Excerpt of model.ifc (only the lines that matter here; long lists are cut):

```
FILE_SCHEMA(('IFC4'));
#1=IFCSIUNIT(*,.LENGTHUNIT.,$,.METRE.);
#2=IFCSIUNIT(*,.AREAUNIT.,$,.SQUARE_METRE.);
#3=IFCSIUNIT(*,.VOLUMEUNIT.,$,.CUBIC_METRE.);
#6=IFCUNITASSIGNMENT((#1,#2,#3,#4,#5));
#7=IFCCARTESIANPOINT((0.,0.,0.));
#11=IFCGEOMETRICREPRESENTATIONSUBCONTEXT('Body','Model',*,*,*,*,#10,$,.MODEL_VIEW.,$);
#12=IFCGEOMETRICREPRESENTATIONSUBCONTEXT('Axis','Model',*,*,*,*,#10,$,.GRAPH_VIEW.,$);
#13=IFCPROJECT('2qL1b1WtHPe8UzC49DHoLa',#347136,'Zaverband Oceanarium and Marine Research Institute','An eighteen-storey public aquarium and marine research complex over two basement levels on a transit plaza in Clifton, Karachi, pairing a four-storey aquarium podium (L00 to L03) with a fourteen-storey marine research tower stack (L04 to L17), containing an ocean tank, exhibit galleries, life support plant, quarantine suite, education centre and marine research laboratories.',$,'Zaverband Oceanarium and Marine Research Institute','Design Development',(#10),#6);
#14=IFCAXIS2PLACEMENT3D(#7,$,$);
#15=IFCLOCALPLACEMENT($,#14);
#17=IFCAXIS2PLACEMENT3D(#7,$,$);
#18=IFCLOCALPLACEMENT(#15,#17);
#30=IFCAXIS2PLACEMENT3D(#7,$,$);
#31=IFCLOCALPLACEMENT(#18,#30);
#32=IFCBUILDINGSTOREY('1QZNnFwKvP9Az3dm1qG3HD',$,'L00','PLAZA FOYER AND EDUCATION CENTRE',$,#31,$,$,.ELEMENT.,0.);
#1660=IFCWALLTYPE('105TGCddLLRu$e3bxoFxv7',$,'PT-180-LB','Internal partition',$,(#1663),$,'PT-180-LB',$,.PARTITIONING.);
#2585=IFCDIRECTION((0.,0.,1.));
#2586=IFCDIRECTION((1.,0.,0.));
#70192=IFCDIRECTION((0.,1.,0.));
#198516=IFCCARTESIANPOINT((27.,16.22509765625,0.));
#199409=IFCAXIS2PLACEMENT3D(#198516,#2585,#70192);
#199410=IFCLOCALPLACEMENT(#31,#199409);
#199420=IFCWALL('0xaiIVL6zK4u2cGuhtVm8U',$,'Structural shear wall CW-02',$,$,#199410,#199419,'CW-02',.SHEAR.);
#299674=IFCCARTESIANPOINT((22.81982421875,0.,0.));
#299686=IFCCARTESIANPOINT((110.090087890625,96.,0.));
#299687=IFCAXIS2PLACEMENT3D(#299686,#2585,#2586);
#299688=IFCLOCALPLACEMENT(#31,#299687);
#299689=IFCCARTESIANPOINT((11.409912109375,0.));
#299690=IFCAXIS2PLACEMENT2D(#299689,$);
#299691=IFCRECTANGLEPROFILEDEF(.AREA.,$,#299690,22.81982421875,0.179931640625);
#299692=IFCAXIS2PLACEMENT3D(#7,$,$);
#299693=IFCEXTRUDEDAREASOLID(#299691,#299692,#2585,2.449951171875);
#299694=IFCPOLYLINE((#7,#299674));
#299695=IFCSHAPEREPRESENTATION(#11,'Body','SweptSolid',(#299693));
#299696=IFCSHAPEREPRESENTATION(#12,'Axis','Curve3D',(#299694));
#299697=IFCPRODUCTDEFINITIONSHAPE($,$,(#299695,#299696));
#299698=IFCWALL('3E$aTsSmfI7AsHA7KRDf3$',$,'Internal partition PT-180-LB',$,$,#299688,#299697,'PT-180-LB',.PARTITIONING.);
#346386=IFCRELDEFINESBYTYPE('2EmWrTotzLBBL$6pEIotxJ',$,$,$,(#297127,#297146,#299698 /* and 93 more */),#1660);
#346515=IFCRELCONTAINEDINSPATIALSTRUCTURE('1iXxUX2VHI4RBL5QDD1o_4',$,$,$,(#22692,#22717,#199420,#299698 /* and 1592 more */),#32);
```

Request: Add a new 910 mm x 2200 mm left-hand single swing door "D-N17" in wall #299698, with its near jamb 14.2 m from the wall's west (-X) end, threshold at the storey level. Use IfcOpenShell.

```python
import numpy as np
import ifcopenshell
import ifcopenshell.api.feature
import ifcopenshell.api.geometry
import ifcopenshell.api.root
import ifcopenshell.api.spatial
import ifcopenshell.geom
import ifcopenshell.util.element
import ifcopenshell.util.placement
import ifcopenshell.util.representation
import ifcopenshell.util.shape
import ifcopenshell.util.unit

model = ifcopenshell.open("model.ifc")
unit_scale = ifcopenshell.util.unit.calculate_unit_scale(model)
settings = ifcopenshell.geom.settings()


def volume(element):
    """Net volume in cubic metres, openings subtracted."""
    shape = ifcopenshell.geom.create_shape(settings, element)
    return ifcopenshell.util.shape.get_volume(shape.geometry)


wall = model.by_guid("3E$aTsSmfI7AsHA7KRDf3$")
storey = ifcopenshell.util.element.get_container(wall, ifc_class="IfcBuildingStorey")
context = ifcopenshell.util.representation.get_context(model, "Model", "Body", "MODEL_VIEW")
before = volume(wall)

width, height, from_end, sill = 0.91, 2.2, 14.2, 0.0  # metres

# The wall runs along its own X axis, and the end named is its -X end.
wall_shape = ifcopenshell.geom.create_shape(settings, wall)
x, y, z = ifcopenshell.util.shape.get_vertices(wall_shape.geometry).T
start = x.min() + from_end
face, thickness = float(y.min()), float(y.max() - y.min())
wall_matrix = ifcopenshell.util.placement.get_local_placement(wall.ObjectPlacement)
level = ifcopenshell.util.placement.get_local_placement(storey.ObjectPlacement)[2, 3]


def in_wall(x, y):
    """Placement at x, y metres in the wall's axes, at sill height."""
    matrix = wall_matrix.copy()
    matrix[:, 3] = wall_matrix @ np.array([x / unit_scale, y / unit_scale, 0.0, 1.0])
    matrix[2, 3] = level + sill / unit_scale
    return matrix


# Opening: a box that overshoots both wall faces by 50 mm.
opening = ifcopenshell.api.root.create_entity(model, ifc_class="IfcOpeningElement", predefined_type="OPENING")
box = ifcopenshell.api.geometry.add_wall_representation(
    model, context=context, length=width, height=height, thickness=thickness + 0.1
)
ifcopenshell.api.geometry.assign_representation(model, product=opening, representation=box)
ifcopenshell.api.geometry.edit_object_placement(model, product=opening, matrix=in_wall(start, face - 0.05), is_si=False)
ifcopenshell.api.feature.add_feature(model, feature=opening, element=wall)

door = ifcopenshell.api.root.create_entity(model, ifc_class="IfcDoor", name="D-N17", predefined_type="DOOR")
door.OverallWidth, door.OverallHeight = width / unit_scale, height / unit_scale
door.OperationType = "SINGLE_SWING_LEFT"
body = ifcopenshell.api.geometry.add_door_representation(
    model,
    context=context,
    overall_width=door.OverallWidth,
    overall_height=door.OverallHeight,
    operation_type="SINGLE_SWING_LEFT",
    lining_properties={"LiningDepth": thickness / unit_scale, "ThresholdDepth": thickness / unit_scale},
)
ifcopenshell.api.geometry.assign_representation(model, product=door, representation=body)
ifcopenshell.api.spatial.assign_container(model, products=[door], relating_structure=storey)
ifcopenshell.api.feature.add_filling(model, opening=opening, element=door)

# The lining spans the wall, so the door starts at the wall face.
ifcopenshell.api.geometry.edit_object_placement(model, product=door, matrix=in_wall(start, face), is_si=False)

after = volume(wall)

print(f"wall volume {before:.3f} -> {after:.3f} m3")

model.write("model_edited.ifc")
```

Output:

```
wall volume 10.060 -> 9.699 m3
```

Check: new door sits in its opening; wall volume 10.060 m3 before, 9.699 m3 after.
